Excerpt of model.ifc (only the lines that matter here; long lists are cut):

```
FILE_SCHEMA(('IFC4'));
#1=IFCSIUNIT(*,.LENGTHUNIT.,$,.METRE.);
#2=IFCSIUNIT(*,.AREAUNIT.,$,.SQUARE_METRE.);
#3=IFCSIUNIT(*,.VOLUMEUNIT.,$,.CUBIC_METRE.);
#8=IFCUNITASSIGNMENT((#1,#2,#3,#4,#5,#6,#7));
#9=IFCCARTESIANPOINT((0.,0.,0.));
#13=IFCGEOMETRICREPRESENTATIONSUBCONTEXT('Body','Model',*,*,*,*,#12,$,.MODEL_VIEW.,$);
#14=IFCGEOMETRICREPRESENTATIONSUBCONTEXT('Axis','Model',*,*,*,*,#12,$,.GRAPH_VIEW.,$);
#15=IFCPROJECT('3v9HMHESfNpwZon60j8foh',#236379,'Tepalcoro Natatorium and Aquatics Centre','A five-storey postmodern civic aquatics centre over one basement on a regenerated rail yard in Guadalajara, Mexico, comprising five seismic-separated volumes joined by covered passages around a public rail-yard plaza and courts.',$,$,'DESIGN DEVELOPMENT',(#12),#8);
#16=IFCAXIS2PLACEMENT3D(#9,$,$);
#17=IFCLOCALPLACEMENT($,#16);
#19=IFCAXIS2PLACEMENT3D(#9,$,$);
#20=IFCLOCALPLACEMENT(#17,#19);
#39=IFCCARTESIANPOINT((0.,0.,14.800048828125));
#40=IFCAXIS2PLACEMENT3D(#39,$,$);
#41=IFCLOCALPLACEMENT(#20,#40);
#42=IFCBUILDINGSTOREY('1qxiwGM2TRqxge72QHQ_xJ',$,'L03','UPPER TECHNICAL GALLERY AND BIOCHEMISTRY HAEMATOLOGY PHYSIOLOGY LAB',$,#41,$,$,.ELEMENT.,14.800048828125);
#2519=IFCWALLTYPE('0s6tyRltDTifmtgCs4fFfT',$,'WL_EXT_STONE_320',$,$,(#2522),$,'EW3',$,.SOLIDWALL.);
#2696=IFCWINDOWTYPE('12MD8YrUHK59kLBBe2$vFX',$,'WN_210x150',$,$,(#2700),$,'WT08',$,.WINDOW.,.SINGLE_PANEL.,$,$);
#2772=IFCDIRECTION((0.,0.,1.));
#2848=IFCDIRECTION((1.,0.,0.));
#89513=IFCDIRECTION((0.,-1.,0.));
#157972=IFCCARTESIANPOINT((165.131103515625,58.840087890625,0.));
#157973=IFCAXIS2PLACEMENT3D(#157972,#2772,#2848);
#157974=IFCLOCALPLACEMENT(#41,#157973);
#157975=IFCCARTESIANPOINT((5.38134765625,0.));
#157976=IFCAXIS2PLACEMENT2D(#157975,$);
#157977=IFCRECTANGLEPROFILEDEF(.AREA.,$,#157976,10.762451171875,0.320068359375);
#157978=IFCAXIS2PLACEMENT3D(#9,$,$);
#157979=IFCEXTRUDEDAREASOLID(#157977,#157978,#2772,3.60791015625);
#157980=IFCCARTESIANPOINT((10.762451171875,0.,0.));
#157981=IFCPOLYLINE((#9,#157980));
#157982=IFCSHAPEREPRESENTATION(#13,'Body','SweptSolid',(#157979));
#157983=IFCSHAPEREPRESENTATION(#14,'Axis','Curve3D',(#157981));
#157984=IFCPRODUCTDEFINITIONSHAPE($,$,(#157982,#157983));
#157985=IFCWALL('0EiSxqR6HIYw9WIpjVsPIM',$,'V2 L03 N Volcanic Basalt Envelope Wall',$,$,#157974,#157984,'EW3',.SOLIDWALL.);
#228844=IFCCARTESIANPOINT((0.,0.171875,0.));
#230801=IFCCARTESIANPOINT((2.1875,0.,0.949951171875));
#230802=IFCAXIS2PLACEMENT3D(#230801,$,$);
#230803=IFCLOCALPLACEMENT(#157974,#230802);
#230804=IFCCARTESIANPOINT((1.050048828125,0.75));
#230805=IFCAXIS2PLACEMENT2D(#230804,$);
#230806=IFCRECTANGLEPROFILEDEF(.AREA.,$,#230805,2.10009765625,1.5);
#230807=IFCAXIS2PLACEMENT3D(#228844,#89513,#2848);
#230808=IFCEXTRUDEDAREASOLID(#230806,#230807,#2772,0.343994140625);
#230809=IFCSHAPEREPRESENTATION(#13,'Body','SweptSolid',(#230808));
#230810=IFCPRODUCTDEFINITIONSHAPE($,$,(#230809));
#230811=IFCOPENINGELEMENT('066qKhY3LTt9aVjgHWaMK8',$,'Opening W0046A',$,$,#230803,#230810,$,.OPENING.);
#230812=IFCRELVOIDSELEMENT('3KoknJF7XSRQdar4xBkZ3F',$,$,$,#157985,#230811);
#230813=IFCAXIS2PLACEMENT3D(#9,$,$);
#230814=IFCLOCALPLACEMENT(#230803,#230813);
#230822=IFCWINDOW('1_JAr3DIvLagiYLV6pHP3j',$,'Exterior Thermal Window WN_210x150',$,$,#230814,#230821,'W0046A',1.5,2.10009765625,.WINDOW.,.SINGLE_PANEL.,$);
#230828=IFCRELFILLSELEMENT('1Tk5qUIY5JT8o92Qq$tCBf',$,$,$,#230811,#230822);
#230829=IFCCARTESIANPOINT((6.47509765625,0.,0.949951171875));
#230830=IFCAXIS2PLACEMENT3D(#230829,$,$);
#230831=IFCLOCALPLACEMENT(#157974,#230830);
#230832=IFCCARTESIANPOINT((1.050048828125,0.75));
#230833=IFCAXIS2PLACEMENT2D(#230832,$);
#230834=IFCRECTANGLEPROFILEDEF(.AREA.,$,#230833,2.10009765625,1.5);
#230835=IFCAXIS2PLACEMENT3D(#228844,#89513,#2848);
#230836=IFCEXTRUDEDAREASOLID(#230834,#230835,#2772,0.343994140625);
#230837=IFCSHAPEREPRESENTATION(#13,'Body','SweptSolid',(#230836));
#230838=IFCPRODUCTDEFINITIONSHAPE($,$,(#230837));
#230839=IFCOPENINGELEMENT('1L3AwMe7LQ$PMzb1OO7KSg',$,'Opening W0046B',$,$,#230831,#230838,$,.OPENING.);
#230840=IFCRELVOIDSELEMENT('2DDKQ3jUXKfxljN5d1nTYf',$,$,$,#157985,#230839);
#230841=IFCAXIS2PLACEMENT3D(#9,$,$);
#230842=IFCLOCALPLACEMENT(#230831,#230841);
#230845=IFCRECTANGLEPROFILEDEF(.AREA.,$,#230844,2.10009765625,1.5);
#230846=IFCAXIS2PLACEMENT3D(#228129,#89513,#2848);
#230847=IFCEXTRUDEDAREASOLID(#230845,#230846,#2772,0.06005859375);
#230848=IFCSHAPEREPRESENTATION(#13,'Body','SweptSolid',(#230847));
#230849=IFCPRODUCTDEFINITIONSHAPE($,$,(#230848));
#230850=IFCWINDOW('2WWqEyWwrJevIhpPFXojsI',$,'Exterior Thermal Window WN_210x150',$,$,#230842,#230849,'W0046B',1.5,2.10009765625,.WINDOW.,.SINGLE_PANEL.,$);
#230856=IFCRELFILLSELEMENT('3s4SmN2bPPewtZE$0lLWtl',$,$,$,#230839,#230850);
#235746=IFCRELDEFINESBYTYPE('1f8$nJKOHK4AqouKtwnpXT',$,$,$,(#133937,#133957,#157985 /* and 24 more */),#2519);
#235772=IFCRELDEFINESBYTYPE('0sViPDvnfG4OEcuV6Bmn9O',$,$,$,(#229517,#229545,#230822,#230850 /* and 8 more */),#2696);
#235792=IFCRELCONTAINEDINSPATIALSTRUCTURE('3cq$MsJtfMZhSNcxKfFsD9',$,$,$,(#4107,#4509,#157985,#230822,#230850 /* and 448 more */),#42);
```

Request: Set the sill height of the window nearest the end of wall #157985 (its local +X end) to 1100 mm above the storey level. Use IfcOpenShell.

```python
import numpy as np
import ifcopenshell
import ifcopenshell.api.geometry
import ifcopenshell.geom
import ifcopenshell.util.element
import ifcopenshell.util.placement
import ifcopenshell.util.shape
import ifcopenshell.util.unit

model = ifcopenshell.open("model.ifc")
unit_scale = ifcopenshell.util.unit.calculate_unit_scale(model)

window = model.by_guid("2WWqEyWwrJevIhpPFXojsI")
opening = window.FillsVoids[0].RelatingOpeningElement
storey = ifcopenshell.util.element.get_container(window, ifc_class="IfcBuildingStorey")
level = ifcopenshell.util.placement.get_local_placement(storey.ObjectPlacement)[2, 3]

# The opening's origin need not be at the sill, so measure its lowest point.
shape = ifcopenshell.geom.create_shape(ifcopenshell.geom.settings(), opening)
bottom = ifcopenshell.util.shape.get_shape_bottom_elevation(shape, shape.geometry) / unit_scale
dz = level + 1.1 / unit_scale - bottom

shift = np.array([0.0, 0.0, dz])
# The window is placed relative to its opening, so it follows when the opening moves.
matrix = ifcopenshell.util.placement.get_local_placement(opening.ObjectPlacement)
matrix[:3, 3] += shift
ifcopenshell.api.geometry.edit_object_placement(
    model, product=opening, matrix=matrix, is_si=False, should_transform_children=True
)

print(f"moved by {dz * unit_scale:+.3f} m")

model.write("model_rev.ifc")
```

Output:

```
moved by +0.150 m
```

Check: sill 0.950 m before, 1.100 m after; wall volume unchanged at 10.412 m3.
